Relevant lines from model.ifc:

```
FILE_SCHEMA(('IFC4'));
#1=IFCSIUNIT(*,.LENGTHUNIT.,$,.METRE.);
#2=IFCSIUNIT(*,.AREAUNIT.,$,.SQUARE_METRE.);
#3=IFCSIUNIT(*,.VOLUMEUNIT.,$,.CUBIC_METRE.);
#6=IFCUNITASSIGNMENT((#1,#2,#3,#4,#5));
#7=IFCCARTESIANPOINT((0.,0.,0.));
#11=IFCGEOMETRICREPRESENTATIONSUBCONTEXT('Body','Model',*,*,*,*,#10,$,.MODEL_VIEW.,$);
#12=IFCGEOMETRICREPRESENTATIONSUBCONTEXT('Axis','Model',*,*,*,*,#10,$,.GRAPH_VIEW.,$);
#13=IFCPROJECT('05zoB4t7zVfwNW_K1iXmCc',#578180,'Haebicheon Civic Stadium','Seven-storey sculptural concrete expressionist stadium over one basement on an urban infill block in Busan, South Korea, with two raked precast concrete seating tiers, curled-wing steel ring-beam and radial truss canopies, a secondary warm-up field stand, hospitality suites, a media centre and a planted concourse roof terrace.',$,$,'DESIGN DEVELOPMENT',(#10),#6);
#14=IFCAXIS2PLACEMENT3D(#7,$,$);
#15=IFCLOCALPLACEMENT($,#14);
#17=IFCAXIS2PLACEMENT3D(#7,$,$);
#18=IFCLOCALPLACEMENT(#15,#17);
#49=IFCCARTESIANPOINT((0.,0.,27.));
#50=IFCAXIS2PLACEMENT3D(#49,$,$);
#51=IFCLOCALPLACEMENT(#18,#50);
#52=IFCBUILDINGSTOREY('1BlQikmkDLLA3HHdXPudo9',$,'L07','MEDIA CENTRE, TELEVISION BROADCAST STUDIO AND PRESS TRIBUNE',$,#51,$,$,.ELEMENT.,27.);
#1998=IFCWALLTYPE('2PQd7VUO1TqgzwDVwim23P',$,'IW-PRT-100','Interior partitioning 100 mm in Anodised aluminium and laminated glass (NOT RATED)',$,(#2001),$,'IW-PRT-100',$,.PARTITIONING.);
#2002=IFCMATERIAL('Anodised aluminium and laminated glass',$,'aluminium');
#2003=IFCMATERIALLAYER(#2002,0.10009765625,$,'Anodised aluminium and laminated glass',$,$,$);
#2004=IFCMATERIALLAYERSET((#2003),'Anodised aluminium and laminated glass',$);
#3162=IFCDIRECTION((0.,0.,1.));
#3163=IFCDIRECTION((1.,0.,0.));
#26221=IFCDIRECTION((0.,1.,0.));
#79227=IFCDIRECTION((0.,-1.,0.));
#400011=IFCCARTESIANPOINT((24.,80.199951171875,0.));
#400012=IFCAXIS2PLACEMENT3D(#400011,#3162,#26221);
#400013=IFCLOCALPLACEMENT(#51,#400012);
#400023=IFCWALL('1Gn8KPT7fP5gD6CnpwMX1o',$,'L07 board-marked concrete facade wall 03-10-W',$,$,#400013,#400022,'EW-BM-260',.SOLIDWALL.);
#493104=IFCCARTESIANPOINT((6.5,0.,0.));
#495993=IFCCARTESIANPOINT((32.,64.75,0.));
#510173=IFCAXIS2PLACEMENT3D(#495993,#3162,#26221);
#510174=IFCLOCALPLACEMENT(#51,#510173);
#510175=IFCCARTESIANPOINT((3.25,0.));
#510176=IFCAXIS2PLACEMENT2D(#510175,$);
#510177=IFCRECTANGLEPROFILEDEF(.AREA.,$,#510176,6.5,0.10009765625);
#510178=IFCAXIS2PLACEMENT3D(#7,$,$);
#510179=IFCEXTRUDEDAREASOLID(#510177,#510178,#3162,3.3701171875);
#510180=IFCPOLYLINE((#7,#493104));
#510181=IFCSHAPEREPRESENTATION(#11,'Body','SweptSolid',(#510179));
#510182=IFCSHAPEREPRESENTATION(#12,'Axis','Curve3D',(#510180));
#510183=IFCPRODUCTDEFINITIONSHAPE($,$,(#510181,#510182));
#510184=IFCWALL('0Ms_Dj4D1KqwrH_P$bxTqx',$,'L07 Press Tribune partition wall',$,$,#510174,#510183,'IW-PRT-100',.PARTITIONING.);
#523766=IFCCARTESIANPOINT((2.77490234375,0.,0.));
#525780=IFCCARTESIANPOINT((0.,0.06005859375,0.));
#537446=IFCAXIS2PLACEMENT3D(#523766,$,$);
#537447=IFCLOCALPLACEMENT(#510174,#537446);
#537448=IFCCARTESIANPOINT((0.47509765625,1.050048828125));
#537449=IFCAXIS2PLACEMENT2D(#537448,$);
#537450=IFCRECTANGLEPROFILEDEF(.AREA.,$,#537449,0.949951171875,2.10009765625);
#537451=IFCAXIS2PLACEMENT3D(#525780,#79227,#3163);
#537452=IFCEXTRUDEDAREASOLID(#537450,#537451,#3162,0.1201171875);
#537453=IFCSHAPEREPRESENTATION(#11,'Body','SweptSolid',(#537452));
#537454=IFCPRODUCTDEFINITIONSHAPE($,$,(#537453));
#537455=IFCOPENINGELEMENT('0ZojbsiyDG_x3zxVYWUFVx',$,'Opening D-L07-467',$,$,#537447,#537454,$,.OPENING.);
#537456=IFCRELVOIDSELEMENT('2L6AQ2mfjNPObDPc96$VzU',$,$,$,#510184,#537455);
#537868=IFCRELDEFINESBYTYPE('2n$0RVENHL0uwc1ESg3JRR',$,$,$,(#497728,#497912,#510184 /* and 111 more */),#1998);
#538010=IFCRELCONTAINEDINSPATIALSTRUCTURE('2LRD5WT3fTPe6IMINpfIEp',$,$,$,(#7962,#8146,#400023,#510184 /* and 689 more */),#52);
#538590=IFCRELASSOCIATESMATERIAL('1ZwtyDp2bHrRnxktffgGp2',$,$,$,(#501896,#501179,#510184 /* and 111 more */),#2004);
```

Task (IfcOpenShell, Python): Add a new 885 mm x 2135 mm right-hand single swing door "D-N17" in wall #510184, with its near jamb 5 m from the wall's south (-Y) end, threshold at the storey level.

```python
import numpy as np
import ifcopenshell
import ifcopenshell.api.feature
import ifcopenshell.api.geometry
import ifcopenshell.api.root
import ifcopenshell.api.spatial
import ifcopenshell.geom
import ifcopenshell.util.element
import ifcopenshell.util.placement
import ifcopenshell.util.representation
import ifcopenshell.util.shape
import ifcopenshell.util.unit

model = ifcopenshell.open("model.ifc")
unit_scale = ifcopenshell.util.unit.calculate_unit_scale(model)
settings = ifcopenshell.geom.settings()


def volume(element):
    """Net volume in cubic metres, openings subtracted."""
    shape = ifcopenshell.geom.create_shape(settings, element)
    return ifcopenshell.util.shape.get_volume(shape.geometry)


wall = model.by_id(510184)
storey = ifcopenshell.util.element.get_container(wall, ifc_class="IfcBuildingStorey")
context = ifcopenshell.util.representation.get_context(model, "Model", "Body", "MODEL_VIEW")
before = volume(wall)

width, height, from_end, sill = 0.885, 2.135, 5, 0.0  # metres

# The wall runs along its own X axis, and the end named is its -X end.
wall_shape = ifcopenshell.geom.create_shape(settings, wall)
x, y, z = ifcopenshell.util.shape.get_vertices(wall_shape.geometry).T
start = x.min() + from_end
face, thickness = float(y.min()), float(y.max() - y.min())
wall_matrix = ifcopenshell.util.placement.get_local_placement(wall.ObjectPlacement)
level = ifcopenshell.util.placement.get_local_placement(storey.ObjectPlacement)[2, 3]


def in_wall(x, y):
    """Placement at x, y metres in the wall's axes, at sill height."""
    matrix = wall_matrix.copy()
    matrix[:, 3] = wall_matrix @ np.array([x / unit_scale, y / unit_scale, 0.0, 1.0])
    matrix[2, 3] = level + sill / unit_scale
    return matrix


# Opening: a box that overshoots both wall faces by 50 mm.
opening = ifcopenshell.api.root.create_entity(model, ifc_class="IfcOpeningElement", predefined_type="OPENING")
box = ifcopenshell.api.geometry.add_wall_representation(
    model, context=context, length=width, height=height, thickness=thickness + 0.1
)
ifcopenshell.api.geometry.assign_representation(model, product=opening, representation=box)
ifcopenshell.api.geometry.edit_object_placement(model, product=opening, matrix=in_wall(start, face - 0.05), is_si=False)
ifcopenshell.api.feature.add_feature(model, feature=opening, element=wall)

door = ifcopenshell.api.root.create_entity(model, ifc_class="IfcDoor", name="D-N17", predefined_type="DOOR")
door.OverallWidth, door.OverallHeight = width / unit_scale, height / unit_scale
door.OperationType = "SINGLE_SWING_RIGHT"
body = ifcopenshell.api.geometry.add_door_representation(
    model,
    context=context,
    overall_width=door.OverallWidth,
    overall_height=door.OverallHeight,
    operation_type="SINGLE_SWING_RIGHT",
    lining_properties={"LiningDepth": thickness / unit_scale, "ThresholdDepth": thickness / unit_scale},
)
ifcopenshell.api.geometry.assign_representation(model, product=door, representation=body)
ifcopenshell.api.spatial.assign_container(model, products=[door], relating_structure=storey)
ifcopenshell.api.feature.add_filling(model, opening=opening, element=door)

# The lining spans the wall, so the door starts at the wall face.
ifcopenshell.api.geometry.edit_object_placement(model, product=door, matrix=in_wall(start, face), is_si=False)

after = volume(wall)

print(f"wall volume {before:.3f} -> {after:.3f} m3")

model.write("model_edited.ifc")
```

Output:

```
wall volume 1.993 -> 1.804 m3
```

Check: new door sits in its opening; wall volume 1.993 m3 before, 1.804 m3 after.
